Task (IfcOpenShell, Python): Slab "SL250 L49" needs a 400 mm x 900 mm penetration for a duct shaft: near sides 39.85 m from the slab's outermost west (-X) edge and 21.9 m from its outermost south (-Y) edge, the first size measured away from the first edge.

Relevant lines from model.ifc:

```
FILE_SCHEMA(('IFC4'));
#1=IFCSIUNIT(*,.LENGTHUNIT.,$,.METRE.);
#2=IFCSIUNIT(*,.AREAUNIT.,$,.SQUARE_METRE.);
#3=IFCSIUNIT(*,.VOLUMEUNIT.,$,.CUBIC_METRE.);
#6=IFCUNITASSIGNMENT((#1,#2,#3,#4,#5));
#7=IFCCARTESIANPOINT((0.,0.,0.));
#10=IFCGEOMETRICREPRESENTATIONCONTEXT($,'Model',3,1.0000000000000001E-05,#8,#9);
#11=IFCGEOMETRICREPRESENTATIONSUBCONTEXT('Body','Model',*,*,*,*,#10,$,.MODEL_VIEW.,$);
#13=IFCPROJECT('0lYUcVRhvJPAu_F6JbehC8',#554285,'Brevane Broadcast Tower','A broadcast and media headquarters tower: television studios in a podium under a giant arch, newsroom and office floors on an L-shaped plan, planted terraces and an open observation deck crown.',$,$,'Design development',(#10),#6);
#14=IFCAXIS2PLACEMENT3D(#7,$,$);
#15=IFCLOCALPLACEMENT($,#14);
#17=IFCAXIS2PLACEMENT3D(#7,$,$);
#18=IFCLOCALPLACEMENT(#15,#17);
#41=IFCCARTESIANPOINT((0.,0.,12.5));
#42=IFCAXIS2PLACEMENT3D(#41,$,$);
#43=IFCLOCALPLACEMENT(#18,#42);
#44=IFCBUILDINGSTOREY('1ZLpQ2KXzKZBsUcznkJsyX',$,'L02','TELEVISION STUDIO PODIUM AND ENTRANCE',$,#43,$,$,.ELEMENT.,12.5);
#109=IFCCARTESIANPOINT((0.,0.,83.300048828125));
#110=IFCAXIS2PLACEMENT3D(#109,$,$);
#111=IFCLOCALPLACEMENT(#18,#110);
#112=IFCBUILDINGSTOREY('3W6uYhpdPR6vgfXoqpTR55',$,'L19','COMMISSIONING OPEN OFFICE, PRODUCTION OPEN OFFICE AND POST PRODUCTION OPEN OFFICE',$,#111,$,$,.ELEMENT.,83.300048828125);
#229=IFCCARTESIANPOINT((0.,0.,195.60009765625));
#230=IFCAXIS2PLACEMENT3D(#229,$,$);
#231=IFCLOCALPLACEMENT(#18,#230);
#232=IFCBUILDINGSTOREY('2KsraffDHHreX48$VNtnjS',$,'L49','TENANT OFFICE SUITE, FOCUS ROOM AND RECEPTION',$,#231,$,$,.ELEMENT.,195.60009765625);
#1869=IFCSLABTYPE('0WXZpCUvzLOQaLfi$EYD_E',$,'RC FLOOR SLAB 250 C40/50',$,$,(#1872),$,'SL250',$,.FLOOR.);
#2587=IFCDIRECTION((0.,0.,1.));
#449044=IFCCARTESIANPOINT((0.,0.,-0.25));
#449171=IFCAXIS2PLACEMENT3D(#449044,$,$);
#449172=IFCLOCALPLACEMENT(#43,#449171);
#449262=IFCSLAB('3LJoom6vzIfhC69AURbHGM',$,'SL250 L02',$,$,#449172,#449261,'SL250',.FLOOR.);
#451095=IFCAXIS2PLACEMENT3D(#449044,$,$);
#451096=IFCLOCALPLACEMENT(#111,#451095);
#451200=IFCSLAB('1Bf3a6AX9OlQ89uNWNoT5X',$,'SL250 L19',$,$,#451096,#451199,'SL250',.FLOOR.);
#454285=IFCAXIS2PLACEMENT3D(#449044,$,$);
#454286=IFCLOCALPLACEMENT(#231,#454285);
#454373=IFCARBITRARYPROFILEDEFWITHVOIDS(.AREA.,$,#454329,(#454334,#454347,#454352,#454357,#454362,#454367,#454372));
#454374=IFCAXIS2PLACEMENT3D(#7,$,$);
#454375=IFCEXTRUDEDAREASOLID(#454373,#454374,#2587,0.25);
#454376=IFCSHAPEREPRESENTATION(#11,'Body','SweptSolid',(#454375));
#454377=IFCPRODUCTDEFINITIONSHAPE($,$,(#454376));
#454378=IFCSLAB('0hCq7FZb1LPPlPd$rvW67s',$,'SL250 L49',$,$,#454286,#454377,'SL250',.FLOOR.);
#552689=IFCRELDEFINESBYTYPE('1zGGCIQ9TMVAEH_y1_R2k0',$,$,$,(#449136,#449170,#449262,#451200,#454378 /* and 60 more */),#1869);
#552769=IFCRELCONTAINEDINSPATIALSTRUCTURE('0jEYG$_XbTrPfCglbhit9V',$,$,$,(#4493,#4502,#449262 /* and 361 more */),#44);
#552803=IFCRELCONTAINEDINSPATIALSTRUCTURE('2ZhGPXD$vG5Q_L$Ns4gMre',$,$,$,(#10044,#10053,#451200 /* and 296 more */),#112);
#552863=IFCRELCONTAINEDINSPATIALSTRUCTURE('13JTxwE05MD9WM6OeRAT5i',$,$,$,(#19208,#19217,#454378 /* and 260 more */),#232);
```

```python
import numpy as np
import ifcopenshell
import ifcopenshell.api.feature
import ifcopenshell.api.geometry
import ifcopenshell.api.root
import ifcopenshell.geom
import ifcopenshell.util.placement
import ifcopenshell.util.representation
import ifcopenshell.util.shape
import ifcopenshell.util.unit

model = ifcopenshell.open("model.ifc")
unit_scale = ifcopenshell.util.unit.calculate_unit_scale(model)
settings = ifcopenshell.geom.settings()


def volume(element):
    """Net volume in cubic metres, openings subtracted."""
    shape = ifcopenshell.geom.create_shape(settings, element)
    return ifcopenshell.util.shape.get_volume(shape.geometry)


slab = model.by_guid("0hCq7FZb1LPPlPd$rvW67s")
before = volume(slab)

# Extent in the slab's own axes, in metres. The edges named are its -X and -Y sides.
slab_shape = ifcopenshell.geom.create_shape(settings, slab)
vertices = ifcopenshell.util.shape.get_vertices(slab_shape.geometry)
x_min, y_min, bottom = vertices.min(axis=0)
top = vertices[:, 2].max()

opening = ifcopenshell.api.root.create_entity(model, ifc_class="IfcOpeningElement", name="Duct shaft opening", predefined_type="OPENING")
context = ifcopenshell.util.representation.get_context(model, "Model", "Body", "MODEL_VIEW")
width, depth = 0.4, 0.9
outline = [(0.0, 0.0), (width, 0.0), (width, depth), (0.0, depth), (0.0, 0.0)]
# Overshoot both faces by 50 mm so the cut is clean.
shape = ifcopenshell.api.geometry.add_slab_representation(
    model, context=context, depth=top - bottom + 0.1, polyline=outline
)
ifcopenshell.api.geometry.assign_representation(model, product=opening, representation=shape)

matrix = ifcopenshell.util.placement.get_local_placement(slab.ObjectPlacement)
matrix[:, 3] = matrix @ np.append(np.array([x_min + 39.85, y_min + 21.9, bottom - 0.05]) / unit_scale, 1.0)
ifcopenshell.api.geometry.edit_object_placement(model, product=opening, matrix=matrix, is_si=False)
ifcopenshell.api.feature.add_feature(model, feature=opening, element=slab)

after = volume(slab)

print(f"slab volume {before:.3f} -> {after:.3f} m3")

model.write("model_edited.ifc")
```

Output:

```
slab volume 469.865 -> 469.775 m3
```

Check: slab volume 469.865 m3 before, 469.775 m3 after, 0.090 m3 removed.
